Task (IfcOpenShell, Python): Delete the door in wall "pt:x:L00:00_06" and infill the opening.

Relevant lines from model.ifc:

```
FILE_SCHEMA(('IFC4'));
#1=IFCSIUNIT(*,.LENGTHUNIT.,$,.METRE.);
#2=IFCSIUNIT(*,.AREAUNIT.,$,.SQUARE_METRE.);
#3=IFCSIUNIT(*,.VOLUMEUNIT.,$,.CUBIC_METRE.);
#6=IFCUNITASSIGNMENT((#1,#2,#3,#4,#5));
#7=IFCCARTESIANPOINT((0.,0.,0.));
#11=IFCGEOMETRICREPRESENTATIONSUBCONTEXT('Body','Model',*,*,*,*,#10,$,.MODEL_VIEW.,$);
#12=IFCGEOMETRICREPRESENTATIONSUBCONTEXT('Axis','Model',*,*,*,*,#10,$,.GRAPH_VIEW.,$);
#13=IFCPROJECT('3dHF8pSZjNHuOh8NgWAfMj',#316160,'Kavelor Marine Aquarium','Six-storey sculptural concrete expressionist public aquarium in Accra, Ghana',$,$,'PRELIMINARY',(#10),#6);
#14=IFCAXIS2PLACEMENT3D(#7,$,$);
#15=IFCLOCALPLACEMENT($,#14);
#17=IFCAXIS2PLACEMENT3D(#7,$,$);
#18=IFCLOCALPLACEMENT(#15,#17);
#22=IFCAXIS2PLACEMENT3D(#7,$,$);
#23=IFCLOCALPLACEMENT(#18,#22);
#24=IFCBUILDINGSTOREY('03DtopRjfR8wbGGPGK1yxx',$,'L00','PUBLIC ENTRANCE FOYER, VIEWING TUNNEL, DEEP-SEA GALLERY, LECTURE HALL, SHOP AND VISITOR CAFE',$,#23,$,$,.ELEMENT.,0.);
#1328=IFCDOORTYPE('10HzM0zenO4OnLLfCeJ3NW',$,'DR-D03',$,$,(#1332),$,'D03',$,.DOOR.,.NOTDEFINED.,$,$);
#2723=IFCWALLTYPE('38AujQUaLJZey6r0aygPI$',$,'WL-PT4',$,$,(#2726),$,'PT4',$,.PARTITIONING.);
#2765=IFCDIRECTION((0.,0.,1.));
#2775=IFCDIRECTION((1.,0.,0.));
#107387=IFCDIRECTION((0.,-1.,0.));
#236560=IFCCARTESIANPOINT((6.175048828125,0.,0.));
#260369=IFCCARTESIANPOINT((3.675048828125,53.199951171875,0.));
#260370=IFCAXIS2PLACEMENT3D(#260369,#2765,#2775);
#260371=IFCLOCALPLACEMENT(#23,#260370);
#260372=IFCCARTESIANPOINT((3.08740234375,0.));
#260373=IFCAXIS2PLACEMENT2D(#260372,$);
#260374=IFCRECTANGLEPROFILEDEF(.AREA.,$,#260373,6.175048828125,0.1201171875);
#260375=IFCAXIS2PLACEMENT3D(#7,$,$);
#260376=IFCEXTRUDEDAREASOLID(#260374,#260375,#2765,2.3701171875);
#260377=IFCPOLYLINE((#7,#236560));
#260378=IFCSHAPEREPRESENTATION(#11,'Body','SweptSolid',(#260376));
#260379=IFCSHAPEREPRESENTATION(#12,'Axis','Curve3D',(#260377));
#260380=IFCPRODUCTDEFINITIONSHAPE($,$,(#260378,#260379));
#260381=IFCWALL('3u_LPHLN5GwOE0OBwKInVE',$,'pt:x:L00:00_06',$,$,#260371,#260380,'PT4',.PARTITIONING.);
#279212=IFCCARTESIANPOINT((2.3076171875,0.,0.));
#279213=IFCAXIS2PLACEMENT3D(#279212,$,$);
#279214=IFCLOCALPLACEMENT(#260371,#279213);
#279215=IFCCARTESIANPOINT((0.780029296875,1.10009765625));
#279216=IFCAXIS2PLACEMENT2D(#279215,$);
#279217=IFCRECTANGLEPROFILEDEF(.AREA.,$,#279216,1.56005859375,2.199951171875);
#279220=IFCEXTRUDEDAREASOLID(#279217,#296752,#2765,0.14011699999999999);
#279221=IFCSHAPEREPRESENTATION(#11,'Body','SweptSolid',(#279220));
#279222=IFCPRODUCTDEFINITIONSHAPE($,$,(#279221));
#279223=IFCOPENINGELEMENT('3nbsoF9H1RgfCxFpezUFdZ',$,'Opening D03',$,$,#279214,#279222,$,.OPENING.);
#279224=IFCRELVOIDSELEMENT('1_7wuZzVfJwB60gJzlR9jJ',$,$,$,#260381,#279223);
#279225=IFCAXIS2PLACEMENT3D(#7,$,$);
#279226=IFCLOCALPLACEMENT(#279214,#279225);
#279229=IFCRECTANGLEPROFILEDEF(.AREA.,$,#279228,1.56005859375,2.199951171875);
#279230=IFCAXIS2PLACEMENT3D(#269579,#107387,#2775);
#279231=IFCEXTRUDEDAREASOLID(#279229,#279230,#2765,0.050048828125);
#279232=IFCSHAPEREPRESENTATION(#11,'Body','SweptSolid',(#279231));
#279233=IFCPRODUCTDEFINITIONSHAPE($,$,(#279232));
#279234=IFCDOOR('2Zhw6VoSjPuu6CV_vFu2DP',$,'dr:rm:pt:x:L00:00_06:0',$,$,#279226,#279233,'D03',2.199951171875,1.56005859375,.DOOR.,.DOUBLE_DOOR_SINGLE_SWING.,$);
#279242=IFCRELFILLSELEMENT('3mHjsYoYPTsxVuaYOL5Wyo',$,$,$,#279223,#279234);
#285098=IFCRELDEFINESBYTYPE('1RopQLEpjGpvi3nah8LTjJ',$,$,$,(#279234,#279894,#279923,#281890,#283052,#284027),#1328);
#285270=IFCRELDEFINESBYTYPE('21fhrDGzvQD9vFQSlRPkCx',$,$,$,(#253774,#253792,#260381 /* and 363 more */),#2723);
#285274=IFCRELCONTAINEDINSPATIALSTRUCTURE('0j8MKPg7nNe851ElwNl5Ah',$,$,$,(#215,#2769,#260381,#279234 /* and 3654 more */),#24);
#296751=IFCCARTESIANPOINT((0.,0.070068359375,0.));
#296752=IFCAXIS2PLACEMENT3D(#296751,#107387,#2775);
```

```python
import ifcopenshell
import ifcopenshell.api.feature
import ifcopenshell.api.root
import ifcopenshell.geom
import ifcopenshell.util.shape

model = ifcopenshell.open("model.ifc")
settings = ifcopenshell.geom.settings()


def volume(element):
    """Net volume in cubic metres, openings subtracted."""
    shape = ifcopenshell.geom.create_shape(settings, element)
    return ifcopenshell.util.shape.get_volume(shape.geometry)


door = model.by_guid("2Zhw6VoSjPuu6CV_vFu2DP")
opening = door.FillsVoids[0].RelatingOpeningElement
wall = opening.VoidsElements[0].RelatingBuildingElement
before = volume(wall)

ifcopenshell.api.root.remove_product(model, product=door)
ifcopenshell.api.feature.remove_feature(model, feature=opening)

after = volume(wall)

print(f"wall volume {before:.3f} -> {after:.3f} m3")

model.write("model_v2.ifc")
```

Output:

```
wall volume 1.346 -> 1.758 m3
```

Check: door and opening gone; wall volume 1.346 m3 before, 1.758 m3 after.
